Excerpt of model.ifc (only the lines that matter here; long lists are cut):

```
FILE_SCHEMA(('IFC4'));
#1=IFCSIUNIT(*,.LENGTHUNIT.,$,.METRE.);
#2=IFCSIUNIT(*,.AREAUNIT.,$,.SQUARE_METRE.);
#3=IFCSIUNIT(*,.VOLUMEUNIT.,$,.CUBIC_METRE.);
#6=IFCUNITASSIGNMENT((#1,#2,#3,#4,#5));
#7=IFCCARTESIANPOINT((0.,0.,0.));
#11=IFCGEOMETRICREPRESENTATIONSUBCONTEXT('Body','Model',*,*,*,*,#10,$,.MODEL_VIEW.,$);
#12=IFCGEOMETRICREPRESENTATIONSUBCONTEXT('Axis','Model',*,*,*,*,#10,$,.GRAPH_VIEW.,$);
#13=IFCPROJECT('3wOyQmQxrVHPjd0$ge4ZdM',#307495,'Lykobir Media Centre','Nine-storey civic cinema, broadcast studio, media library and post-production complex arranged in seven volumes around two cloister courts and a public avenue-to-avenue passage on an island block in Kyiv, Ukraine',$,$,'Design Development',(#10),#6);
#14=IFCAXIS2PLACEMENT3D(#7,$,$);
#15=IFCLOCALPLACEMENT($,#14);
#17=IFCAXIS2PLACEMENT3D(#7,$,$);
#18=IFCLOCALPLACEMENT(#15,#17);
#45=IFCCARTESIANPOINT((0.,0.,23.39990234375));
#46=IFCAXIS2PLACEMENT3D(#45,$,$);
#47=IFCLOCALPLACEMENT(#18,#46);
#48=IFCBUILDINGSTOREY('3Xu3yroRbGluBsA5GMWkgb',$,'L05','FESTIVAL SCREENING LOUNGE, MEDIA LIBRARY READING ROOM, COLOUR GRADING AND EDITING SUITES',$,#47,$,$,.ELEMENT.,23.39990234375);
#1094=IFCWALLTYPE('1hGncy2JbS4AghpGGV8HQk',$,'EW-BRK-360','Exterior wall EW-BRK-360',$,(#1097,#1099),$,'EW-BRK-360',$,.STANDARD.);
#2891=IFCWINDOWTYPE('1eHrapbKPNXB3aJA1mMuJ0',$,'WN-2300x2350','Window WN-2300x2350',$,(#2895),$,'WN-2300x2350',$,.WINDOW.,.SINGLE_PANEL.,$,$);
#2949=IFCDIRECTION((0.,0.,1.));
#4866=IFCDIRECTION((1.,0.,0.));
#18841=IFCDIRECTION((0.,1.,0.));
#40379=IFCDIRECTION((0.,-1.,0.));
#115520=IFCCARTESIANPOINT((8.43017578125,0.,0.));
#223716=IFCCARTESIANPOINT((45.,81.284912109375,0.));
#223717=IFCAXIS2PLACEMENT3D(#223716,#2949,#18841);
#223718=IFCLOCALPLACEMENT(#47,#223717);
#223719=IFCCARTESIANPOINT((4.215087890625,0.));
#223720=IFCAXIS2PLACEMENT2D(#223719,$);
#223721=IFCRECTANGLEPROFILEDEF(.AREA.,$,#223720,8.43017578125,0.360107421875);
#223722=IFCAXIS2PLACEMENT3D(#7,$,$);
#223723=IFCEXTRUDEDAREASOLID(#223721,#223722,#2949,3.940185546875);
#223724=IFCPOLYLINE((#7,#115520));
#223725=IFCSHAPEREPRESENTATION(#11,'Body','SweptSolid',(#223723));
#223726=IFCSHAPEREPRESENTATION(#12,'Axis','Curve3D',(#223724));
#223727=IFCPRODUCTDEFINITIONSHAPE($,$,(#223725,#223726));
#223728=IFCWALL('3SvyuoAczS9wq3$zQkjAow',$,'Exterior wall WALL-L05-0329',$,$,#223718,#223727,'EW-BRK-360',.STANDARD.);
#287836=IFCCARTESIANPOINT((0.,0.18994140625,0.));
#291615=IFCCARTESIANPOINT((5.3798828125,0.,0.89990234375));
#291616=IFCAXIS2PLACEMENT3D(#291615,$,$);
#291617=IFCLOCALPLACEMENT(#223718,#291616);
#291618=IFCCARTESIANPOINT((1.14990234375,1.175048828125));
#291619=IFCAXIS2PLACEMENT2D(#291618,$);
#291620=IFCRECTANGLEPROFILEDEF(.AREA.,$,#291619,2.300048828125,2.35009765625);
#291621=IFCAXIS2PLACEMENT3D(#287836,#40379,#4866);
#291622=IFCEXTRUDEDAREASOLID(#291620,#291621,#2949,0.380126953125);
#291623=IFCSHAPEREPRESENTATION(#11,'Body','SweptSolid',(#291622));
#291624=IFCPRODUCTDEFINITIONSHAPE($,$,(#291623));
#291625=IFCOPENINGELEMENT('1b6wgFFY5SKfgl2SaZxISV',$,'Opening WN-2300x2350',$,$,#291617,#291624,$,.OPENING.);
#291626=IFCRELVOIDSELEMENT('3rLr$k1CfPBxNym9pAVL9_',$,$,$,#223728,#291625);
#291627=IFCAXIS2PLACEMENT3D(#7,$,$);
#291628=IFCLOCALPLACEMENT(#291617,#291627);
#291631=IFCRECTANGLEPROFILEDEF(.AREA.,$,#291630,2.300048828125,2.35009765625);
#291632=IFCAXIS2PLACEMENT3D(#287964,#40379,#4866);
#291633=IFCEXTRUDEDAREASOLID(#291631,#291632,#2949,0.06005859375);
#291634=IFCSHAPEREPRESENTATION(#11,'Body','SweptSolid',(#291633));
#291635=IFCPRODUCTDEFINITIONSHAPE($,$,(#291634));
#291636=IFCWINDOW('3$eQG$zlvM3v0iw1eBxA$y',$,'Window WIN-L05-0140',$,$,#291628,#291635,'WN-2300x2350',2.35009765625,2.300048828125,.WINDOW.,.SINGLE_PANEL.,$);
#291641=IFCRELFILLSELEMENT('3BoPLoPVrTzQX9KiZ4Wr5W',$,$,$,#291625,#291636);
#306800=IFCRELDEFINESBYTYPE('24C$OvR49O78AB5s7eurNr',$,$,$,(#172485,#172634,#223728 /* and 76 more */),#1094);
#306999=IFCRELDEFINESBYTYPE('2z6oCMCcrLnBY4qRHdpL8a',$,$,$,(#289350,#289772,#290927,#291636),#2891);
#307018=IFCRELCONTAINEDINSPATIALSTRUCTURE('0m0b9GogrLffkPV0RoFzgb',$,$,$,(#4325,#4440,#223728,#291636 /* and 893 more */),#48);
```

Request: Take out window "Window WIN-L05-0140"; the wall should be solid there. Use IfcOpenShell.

```python
import ifcopenshell
import ifcopenshell.api.feature
import ifcopenshell.api.root
import ifcopenshell.geom
import ifcopenshell.util.shape

model = ifcopenshell.open("model.ifc")
settings = ifcopenshell.geom.settings()


def volume(element):
    """Net volume in cubic metres, openings subtracted."""
    shape = ifcopenshell.geom.create_shape(settings, element)
    return ifcopenshell.util.shape.get_volume(shape.geometry)


window = model.by_guid("3$eQG$zlvM3v0iw1eBxA$y")
opening = window.FillsVoids[0].RelatingOpeningElement
wall = opening.VoidsElements[0].RelatingBuildingElement
before = volume(wall)

ifcopenshell.api.root.remove_product(model, product=window)
ifcopenshell.api.feature.remove_feature(model, feature=opening)

after = volume(wall)

print(f"wall volume {before:.3f} -> {after:.3f} m3")

model.write("model-out.ifc")
```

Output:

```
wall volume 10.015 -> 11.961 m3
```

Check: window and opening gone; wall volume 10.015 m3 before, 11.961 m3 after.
